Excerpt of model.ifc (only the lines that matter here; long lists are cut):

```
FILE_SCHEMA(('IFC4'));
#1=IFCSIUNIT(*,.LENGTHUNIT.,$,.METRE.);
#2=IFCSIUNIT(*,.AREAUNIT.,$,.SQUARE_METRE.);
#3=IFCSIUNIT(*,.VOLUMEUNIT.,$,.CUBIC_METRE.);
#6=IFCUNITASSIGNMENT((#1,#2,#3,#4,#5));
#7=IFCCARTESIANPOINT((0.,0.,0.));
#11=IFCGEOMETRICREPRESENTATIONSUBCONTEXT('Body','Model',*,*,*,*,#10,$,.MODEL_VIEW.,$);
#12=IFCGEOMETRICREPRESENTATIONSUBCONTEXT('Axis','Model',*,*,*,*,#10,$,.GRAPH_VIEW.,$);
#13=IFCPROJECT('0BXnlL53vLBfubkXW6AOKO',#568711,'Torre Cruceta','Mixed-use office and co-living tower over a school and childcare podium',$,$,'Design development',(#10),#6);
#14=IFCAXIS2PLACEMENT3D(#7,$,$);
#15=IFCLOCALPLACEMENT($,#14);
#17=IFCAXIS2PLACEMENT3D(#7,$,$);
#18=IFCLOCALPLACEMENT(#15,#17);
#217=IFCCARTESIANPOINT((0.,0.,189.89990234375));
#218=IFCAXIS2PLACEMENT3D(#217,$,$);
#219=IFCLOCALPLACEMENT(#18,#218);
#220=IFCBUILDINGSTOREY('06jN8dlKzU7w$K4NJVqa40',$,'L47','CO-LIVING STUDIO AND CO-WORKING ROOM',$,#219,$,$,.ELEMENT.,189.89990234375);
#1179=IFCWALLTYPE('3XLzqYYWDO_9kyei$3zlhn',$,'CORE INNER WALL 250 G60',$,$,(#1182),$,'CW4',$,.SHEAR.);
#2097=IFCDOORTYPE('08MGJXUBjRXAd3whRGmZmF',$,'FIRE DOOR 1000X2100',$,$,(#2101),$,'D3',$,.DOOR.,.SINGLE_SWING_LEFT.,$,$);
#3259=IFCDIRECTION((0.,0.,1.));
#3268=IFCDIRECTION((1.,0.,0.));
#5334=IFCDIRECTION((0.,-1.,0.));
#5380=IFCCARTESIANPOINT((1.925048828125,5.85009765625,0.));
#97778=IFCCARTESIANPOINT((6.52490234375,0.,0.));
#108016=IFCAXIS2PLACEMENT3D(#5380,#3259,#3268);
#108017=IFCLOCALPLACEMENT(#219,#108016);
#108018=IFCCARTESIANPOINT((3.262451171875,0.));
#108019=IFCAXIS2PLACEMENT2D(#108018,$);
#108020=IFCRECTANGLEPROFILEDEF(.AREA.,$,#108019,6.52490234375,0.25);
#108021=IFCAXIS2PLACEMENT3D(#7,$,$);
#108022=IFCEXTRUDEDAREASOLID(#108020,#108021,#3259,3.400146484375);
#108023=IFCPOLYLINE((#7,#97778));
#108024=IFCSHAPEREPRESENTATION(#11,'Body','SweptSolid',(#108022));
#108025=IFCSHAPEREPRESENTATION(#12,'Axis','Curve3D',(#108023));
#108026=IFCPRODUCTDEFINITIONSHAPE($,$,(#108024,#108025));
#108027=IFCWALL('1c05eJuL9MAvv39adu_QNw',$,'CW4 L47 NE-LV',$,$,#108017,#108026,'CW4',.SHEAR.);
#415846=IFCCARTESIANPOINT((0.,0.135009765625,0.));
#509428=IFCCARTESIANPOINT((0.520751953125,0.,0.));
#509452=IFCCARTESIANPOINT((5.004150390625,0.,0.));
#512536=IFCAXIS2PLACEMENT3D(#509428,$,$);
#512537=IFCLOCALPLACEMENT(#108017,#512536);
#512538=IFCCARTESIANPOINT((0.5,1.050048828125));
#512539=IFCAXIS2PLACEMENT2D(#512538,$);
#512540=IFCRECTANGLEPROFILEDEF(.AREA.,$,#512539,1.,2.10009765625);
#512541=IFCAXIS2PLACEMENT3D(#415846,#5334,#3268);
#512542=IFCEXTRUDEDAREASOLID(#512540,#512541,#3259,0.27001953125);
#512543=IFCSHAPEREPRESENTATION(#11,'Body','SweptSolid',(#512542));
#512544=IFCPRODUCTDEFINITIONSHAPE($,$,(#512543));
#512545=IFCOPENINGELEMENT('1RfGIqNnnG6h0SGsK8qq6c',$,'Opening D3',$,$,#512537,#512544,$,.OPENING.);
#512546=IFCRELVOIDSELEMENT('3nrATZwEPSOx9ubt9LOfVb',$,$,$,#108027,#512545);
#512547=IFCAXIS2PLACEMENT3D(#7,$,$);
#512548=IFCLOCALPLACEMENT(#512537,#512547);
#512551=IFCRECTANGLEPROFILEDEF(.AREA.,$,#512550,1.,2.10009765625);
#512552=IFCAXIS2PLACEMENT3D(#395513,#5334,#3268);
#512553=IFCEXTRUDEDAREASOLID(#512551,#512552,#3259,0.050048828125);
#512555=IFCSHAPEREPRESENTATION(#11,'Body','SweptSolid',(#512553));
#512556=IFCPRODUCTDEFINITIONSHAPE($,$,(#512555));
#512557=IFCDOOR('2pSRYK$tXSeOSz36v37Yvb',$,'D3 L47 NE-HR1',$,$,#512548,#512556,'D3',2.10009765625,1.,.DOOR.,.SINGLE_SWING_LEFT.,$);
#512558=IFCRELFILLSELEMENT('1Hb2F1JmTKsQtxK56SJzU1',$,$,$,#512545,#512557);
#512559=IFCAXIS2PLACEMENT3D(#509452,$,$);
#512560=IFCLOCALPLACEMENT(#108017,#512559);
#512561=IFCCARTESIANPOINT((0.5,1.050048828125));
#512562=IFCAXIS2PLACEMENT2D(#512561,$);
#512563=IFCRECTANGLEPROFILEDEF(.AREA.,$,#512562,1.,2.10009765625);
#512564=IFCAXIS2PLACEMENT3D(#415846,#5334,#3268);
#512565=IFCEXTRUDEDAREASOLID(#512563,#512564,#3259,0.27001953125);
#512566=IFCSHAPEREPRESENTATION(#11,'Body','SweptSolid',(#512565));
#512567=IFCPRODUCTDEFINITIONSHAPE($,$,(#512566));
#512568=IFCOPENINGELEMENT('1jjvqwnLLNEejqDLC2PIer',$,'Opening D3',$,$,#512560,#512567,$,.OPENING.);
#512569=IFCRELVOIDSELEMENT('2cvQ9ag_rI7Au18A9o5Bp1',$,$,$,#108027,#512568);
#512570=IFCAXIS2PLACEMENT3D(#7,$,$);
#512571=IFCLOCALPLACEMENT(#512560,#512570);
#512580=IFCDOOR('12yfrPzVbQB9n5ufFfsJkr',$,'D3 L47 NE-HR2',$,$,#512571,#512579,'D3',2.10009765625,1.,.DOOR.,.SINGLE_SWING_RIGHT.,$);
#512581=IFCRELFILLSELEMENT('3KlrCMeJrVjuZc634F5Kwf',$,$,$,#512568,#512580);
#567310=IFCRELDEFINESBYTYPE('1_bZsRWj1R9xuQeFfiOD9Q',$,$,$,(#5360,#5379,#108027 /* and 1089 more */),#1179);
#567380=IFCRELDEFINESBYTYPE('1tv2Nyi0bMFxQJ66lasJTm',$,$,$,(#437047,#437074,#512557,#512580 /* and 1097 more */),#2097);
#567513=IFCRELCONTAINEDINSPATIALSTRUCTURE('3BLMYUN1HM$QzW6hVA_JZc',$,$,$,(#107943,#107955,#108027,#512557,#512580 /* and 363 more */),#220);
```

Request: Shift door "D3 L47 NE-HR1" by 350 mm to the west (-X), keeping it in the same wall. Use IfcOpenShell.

```python
import ifcopenshell
import ifcopenshell.api.geometry
import ifcopenshell.util.placement
import ifcopenshell.util.unit

model = ifcopenshell.open("model.ifc")
unit_scale = ifcopenshell.util.unit.calculate_unit_scale(model)

door = model.by_guid("2pSRYK$tXSeOSz36v37Yvb")
opening = door.FillsVoids[0].RelatingOpeningElement
wall = opening.VoidsElements[0].RelatingBuildingElement

wall_matrix = ifcopenshell.util.placement.get_local_placement(wall.ObjectPlacement)
shift = wall_matrix[:3, 0] * -0.35 / unit_scale
before = ifcopenshell.util.placement.get_local_placement(door.ObjectPlacement)[:3, 3].copy()

# The door is placed relative to its opening, so it follows when the opening moves.
matrix = ifcopenshell.util.placement.get_local_placement(opening.ObjectPlacement)
matrix[:3, 3] += shift
ifcopenshell.api.geometry.edit_object_placement(
    model, product=opening, matrix=matrix, is_si=False, should_transform_children=True
)

after = ifcopenshell.util.placement.get_local_placement(door.ObjectPlacement)[:3, 3]
print("door moved by", (after - before).round(3) + 0.0)

model.write("model-out.ifc")
```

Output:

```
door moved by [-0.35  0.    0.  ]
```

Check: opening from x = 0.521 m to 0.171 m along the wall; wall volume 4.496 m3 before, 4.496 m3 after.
